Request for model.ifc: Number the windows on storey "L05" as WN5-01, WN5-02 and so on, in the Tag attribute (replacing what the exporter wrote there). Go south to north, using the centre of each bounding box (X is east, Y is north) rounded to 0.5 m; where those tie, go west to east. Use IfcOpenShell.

First a look at what the model holds.

```python
import ifcopenshell
import ifcopenshell.util.element
import ifcopenshell.util.placement

model = ifcopenshell.open("model.ifc")
print(model.schema)
storey = next(s for s in model.by_type("IfcBuildingStorey") if s.Name == "L05")
windows = [e for e in ifcopenshell.util.element.get_decomposition(storey) if e.is_a("IfcWindow")]
for e in sorted(windows, key=lambda e: e.id()):
    origin = ifcopenshell.util.placement.get_local_placement(e.ObjectPlacement)[:3, 3]
    print(e.id(), e.Tag, e.Name, origin.round(2) + 0.0, sep=" | ")
```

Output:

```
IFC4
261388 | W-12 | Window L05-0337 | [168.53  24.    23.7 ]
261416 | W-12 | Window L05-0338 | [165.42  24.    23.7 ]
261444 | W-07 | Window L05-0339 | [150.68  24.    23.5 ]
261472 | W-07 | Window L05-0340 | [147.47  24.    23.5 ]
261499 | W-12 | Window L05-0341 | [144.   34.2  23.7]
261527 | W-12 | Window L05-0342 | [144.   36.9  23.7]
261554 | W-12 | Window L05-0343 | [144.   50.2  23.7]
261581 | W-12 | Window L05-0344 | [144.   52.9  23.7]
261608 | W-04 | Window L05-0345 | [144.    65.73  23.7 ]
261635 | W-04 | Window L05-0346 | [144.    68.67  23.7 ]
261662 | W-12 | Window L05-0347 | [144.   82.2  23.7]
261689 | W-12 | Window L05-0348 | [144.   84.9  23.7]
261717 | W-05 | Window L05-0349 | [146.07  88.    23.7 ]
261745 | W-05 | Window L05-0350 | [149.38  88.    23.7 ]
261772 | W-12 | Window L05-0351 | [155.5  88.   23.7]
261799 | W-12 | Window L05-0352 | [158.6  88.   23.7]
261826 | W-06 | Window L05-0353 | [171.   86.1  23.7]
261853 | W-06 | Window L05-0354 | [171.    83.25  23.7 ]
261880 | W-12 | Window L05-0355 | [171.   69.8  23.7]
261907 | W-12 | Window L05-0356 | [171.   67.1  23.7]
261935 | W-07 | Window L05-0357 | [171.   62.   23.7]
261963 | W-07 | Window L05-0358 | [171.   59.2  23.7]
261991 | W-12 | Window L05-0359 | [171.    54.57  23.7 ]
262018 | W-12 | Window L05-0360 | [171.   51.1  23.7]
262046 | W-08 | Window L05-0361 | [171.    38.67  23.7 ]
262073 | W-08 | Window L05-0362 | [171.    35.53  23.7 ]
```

```python
import ifcopenshell
import ifcopenshell.geom
import ifcopenshell.util.element
import ifcopenshell.util.shape

model = ifcopenshell.open("model.ifc")
settings = ifcopenshell.geom.settings()
settings.set("use-world-coords", True)


def centre(element):
    shape = ifcopenshell.geom.create_shape(settings, element)
    return ifcopenshell.util.shape.get_bbox_centroid(shape.geometry)


storey = next(s for s in model.by_type("IfcBuildingStorey") if s.Name == "L05")
windows = [e for e in ifcopenshell.util.element.get_decomposition(storey) if e.is_a("IfcWindow")]

# Insertion points can sit at a corner or the storey origin, so sort by the geometry (in metres).
centres = {e: centre(e) for e in windows}
windows.sort(key=lambda e: (round(centres[e][1] / 0.5), centres[e][0]))

for i, e in enumerate(windows, start=1):
    number = f"WN5-{i:02d}"
    e.Tag = number
    print(e.id(), number)

model.write("model_edited.ifc")
```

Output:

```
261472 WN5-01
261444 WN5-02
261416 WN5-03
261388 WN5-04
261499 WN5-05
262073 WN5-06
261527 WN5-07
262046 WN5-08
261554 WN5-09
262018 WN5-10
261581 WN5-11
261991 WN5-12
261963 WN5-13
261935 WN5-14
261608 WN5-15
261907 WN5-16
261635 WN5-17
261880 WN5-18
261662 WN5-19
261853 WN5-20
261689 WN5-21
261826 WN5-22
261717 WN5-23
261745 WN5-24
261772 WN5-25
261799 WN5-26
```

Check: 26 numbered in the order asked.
